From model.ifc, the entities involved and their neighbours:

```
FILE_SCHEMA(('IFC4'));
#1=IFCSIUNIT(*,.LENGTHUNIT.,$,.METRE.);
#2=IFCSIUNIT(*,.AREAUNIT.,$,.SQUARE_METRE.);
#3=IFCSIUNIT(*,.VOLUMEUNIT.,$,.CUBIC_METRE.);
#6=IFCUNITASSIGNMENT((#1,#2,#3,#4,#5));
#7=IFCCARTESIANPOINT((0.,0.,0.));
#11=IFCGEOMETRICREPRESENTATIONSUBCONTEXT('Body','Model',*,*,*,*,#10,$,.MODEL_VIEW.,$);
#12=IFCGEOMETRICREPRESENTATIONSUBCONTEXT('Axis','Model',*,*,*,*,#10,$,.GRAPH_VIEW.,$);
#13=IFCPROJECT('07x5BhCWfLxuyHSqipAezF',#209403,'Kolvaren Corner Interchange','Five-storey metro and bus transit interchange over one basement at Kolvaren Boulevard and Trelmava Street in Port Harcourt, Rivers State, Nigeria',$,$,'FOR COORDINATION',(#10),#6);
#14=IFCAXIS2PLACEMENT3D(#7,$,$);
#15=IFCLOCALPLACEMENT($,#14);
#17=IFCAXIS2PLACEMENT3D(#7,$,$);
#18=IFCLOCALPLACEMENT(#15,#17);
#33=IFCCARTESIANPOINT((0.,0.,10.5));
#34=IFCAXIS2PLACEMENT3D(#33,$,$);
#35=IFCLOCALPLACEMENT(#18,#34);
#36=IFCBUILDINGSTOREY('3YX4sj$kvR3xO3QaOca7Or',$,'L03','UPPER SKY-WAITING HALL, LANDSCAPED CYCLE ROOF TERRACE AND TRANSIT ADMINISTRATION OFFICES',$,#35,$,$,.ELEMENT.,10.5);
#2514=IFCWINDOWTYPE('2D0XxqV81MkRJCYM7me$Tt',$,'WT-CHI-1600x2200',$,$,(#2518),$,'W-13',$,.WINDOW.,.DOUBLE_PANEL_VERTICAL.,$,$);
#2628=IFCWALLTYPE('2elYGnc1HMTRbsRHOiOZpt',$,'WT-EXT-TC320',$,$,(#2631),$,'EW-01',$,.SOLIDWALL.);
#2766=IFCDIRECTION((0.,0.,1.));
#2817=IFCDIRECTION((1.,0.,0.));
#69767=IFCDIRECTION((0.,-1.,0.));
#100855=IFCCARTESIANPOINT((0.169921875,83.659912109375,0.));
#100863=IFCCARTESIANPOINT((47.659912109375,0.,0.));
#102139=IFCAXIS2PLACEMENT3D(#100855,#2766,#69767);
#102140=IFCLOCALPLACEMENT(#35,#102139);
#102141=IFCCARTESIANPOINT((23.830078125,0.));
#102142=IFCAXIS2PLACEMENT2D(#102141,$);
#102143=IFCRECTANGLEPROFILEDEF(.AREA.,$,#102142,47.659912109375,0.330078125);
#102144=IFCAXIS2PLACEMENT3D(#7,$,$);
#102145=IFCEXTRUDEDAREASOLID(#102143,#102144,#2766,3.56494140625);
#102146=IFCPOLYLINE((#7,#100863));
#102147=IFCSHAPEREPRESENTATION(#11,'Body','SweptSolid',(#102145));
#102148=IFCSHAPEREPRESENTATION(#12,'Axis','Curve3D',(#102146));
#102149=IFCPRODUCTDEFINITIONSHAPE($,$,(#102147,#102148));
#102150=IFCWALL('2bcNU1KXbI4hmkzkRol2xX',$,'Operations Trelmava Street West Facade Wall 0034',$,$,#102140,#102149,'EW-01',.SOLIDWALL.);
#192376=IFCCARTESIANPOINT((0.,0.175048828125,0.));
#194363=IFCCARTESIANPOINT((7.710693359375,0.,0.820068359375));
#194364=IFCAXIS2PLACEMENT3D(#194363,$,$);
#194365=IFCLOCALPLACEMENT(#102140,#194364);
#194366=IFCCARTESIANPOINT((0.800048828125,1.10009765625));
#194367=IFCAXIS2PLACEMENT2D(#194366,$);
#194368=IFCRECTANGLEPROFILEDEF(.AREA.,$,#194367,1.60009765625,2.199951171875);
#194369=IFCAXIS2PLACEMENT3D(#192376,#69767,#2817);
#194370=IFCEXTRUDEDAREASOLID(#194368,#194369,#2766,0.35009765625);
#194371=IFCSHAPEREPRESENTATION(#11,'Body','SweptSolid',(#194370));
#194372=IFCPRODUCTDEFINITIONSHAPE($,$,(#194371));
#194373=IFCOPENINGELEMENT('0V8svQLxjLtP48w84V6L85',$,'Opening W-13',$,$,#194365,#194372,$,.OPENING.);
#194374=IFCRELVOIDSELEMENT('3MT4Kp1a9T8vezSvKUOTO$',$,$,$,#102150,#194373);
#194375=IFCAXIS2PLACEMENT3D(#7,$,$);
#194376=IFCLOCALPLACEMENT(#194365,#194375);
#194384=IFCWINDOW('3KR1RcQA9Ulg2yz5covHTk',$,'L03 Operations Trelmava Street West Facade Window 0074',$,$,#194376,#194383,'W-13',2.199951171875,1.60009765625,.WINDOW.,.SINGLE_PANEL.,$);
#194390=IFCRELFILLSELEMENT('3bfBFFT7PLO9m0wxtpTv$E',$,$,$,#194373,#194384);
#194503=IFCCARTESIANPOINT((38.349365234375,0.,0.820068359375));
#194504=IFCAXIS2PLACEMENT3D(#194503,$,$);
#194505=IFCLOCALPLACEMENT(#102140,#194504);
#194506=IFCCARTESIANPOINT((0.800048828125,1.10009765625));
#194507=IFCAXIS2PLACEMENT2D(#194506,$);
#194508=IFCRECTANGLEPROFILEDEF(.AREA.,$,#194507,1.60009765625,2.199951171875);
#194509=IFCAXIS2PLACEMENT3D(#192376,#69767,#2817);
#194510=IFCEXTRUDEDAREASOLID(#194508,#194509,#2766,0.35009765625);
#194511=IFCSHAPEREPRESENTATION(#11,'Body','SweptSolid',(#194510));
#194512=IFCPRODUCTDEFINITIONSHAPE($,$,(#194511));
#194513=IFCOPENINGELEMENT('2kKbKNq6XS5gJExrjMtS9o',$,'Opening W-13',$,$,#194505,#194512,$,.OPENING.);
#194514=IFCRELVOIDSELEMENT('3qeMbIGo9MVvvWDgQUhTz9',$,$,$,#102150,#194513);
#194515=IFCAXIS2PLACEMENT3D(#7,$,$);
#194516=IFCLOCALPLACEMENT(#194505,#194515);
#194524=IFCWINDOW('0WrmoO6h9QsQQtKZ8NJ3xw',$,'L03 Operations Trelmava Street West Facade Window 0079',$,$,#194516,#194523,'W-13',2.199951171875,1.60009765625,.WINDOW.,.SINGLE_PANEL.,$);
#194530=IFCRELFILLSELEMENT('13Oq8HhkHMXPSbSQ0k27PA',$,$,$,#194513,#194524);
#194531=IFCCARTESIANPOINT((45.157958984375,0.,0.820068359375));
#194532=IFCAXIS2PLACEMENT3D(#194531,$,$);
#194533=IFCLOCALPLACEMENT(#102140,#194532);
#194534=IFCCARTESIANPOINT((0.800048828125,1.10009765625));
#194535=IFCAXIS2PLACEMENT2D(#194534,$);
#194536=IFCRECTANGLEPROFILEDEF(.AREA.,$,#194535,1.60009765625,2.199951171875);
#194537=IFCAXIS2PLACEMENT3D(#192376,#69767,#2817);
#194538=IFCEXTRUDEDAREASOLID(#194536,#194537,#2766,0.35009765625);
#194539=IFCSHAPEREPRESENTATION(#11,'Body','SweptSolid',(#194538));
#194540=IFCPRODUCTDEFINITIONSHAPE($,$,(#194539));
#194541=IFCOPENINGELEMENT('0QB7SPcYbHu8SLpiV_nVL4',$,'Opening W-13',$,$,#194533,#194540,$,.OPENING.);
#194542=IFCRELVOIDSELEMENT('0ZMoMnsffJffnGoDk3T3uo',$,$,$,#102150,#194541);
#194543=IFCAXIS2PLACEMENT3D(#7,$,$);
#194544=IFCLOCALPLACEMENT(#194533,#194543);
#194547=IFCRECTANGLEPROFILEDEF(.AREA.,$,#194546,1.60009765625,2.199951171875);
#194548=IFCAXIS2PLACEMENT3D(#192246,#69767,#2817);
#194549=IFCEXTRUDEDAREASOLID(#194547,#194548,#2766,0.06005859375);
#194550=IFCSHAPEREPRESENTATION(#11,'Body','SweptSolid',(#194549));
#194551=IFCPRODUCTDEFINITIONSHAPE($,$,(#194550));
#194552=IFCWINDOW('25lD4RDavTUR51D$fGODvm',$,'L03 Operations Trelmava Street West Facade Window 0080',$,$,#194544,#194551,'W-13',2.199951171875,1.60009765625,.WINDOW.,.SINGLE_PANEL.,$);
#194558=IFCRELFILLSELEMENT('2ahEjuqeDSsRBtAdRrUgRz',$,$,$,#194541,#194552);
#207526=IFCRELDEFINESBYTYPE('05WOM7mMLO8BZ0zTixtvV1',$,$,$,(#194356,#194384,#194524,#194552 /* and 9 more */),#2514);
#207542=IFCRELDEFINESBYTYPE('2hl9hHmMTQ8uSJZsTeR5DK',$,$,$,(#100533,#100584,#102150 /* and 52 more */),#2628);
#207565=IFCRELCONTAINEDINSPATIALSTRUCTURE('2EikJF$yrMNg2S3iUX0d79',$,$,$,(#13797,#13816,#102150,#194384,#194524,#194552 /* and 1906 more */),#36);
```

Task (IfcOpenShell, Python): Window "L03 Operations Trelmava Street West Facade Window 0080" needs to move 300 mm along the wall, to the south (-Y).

```python
import ifcopenshell
import ifcopenshell.api.geometry
import ifcopenshell.util.placement
import ifcopenshell.util.unit

model = ifcopenshell.open("model.ifc")
unit_scale = ifcopenshell.util.unit.calculate_unit_scale(model)

window = model.by_guid("25lD4RDavTUR51D$fGODvm")
opening = window.FillsVoids[0].RelatingOpeningElement
wall = opening.VoidsElements[0].RelatingBuildingElement

wall_matrix = ifcopenshell.util.placement.get_local_placement(wall.ObjectPlacement)
shift = wall_matrix[:3, 0] * 0.3 / unit_scale
before = ifcopenshell.util.placement.get_local_placement(window.ObjectPlacement)[:3, 3].copy()

# The window is placed relative to its opening, so it follows when the opening moves.
matrix = ifcopenshell.util.placement.get_local_placement(opening.ObjectPlacement)
matrix[:3, 3] += shift
ifcopenshell.api.geometry.edit_object_placement(
    model, product=opening, matrix=matrix, is_si=False, should_transform_children=True
)

after = ifcopenshell.util.placement.get_local_placement(window.ObjectPlacement)[:3, 3]
print("window moved by", (after - before).round(3) + 0.0)

model.write("model_updated.ifc")
```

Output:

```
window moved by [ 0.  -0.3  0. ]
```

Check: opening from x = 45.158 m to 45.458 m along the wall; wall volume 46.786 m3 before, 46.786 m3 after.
